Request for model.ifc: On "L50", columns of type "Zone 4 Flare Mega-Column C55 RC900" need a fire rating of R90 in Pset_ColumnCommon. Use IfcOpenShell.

First a look at what the model holds.

```python
import ifcopenshell
import ifcopenshell.util.element

model = ifcopenshell.open("model.ifc")
print(model.schema)
storey = next(s for s in model.by_type("IfcBuildingStorey") if s.Name == "L50")
columns = [e for e in ifcopenshell.util.element.get_decomposition(storey) if e.is_a("IfcColumn")]
seen = {}
for e in columns:
    element_type = ifcopenshell.util.element.get_type(e)
    key = (element_type.Name if element_type != e and element_type else None, ifcopenshell.util.element.get_pset(e, "Pset_ColumnCommon", "FireRating"))
    seen[key] = seen.get(key, 0) + 1
for (name, value), count in sorted(seen.items(), key=str):
    print(count, "x", name, "|", value)
```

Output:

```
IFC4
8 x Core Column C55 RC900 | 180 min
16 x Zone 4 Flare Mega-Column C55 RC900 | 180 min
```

```python
import ifcopenshell
import ifcopenshell.api.pset
import ifcopenshell.util.element

model = ifcopenshell.open("model.ifc")

storey = next(s for s in model.by_type("IfcBuildingStorey") if s.Name == "L50")
columns = [e for e in ifcopenshell.util.element.get_decomposition(storey) if e.is_a("IfcColumn")]

count = 0
for e in columns:
    element_type = ifcopenshell.util.element.get_type(e)
    if element_type in (None, e) or element_type.Name != "Zone 4 Flare Mega-Column C55 RC900":
        continue
    found = ifcopenshell.util.element.get_pset(e, "Pset_ColumnCommon", should_inherit=False)
    if found:
        pset = model.by_id(found["id"])
        if len(ifcopenshell.util.element.get_elements_by_pset(pset)) > 1:
            pset = ifcopenshell.api.pset.unshare_pset(model, products=[e], pset=pset)[0]
    else:
        pset = ifcopenshell.api.pset.add_pset(model, product=e, name="Pset_ColumnCommon")
    ifcopenshell.api.pset.edit_pset(model, pset=pset, properties={"FireRating": "R90"})
    count += 1

print(count, "columns updated")

model.write("model_rev.ifc")
```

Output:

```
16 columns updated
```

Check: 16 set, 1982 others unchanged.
